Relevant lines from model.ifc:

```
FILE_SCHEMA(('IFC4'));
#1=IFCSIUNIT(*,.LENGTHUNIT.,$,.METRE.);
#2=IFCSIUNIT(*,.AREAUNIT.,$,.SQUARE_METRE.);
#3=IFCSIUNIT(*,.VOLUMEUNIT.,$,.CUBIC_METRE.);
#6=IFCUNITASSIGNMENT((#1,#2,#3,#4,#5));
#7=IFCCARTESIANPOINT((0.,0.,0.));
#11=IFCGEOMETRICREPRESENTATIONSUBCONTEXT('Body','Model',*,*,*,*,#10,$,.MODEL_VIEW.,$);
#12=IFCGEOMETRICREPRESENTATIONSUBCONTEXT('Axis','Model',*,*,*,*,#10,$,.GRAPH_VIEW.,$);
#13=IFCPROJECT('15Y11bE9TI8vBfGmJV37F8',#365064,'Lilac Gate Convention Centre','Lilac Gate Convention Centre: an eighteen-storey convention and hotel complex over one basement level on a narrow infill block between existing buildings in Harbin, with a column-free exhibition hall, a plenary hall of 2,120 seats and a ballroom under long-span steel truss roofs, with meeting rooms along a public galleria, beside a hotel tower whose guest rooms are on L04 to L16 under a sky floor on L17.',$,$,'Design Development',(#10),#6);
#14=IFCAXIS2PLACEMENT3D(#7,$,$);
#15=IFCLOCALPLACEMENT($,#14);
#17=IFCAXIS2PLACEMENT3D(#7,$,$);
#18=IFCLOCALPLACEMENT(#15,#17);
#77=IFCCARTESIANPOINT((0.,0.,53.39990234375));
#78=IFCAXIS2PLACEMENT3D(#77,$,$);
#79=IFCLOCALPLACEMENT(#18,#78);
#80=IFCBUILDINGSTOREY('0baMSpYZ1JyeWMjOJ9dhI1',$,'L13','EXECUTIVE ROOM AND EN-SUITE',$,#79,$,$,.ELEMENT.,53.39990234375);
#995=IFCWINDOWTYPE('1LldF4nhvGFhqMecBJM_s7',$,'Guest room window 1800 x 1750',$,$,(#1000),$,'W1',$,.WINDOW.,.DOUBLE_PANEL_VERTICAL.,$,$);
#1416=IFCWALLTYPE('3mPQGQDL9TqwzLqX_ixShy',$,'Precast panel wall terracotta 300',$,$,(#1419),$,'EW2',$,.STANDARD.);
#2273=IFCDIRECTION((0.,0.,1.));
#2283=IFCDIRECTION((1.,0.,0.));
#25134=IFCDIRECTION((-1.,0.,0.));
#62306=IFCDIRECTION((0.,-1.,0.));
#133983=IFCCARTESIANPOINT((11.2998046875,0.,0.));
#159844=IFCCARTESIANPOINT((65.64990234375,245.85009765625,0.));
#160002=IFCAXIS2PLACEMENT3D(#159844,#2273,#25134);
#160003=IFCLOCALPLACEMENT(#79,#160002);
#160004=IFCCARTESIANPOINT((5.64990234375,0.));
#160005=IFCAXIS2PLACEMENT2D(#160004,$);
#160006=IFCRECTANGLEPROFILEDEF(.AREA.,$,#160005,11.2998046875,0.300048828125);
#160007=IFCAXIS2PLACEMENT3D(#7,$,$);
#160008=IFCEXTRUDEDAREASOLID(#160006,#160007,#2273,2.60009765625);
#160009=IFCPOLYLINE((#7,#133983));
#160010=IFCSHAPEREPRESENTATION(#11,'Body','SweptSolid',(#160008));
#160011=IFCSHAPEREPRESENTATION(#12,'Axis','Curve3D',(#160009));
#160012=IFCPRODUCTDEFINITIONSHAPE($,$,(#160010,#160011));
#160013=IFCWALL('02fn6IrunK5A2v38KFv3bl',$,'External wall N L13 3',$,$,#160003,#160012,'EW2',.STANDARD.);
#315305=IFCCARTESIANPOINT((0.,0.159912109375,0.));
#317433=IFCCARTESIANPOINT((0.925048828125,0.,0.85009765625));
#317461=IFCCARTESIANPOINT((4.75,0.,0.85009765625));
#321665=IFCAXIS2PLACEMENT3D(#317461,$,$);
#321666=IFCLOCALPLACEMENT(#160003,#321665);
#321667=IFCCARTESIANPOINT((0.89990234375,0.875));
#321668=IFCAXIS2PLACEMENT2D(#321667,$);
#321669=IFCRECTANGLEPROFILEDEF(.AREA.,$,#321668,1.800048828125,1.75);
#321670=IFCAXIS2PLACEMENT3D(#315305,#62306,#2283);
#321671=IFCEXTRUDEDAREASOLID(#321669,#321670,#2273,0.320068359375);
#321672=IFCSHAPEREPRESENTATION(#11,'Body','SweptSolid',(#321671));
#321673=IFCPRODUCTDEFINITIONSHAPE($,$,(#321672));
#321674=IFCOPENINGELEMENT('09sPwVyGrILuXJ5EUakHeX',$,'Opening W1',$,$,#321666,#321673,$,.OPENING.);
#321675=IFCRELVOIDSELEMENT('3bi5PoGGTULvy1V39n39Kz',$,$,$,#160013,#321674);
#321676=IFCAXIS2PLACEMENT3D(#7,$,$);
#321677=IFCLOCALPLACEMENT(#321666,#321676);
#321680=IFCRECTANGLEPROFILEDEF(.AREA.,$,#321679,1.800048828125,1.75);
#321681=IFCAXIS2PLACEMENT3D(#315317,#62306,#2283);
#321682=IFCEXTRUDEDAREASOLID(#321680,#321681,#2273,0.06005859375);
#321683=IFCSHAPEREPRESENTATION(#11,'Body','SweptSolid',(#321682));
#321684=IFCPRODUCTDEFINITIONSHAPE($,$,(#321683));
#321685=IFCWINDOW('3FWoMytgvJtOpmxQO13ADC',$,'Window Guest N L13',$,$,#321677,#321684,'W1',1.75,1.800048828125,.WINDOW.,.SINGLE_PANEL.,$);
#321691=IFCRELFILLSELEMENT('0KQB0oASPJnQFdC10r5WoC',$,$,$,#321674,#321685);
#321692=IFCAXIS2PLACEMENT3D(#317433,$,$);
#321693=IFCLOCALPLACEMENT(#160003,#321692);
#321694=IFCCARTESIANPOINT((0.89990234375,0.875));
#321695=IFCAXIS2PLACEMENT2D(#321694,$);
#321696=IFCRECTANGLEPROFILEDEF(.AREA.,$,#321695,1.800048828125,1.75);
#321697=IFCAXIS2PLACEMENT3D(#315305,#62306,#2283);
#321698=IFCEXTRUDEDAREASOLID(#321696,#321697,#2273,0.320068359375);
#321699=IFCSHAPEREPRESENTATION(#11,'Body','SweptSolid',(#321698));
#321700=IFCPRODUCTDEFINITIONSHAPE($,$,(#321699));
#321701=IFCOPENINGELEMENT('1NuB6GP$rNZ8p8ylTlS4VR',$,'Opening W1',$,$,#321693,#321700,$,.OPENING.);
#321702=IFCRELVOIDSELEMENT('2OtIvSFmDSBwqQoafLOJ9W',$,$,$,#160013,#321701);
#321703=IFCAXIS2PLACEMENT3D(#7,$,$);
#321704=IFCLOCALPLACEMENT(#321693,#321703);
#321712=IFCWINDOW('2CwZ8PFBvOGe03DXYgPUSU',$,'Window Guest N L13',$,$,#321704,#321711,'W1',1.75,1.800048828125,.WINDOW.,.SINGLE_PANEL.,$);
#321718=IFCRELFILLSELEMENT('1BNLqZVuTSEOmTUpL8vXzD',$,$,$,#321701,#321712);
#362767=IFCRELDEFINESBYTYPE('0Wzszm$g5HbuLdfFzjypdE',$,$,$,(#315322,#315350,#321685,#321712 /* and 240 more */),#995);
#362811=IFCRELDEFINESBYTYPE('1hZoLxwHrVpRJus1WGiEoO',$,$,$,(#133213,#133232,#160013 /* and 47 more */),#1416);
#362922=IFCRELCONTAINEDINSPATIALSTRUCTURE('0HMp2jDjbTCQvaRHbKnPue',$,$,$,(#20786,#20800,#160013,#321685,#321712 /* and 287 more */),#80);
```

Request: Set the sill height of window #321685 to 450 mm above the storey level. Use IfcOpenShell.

```python
import numpy as np
import ifcopenshell
import ifcopenshell.api.geometry
import ifcopenshell.geom
import ifcopenshell.util.element
import ifcopenshell.util.placement
import ifcopenshell.util.shape
import ifcopenshell.util.unit

model = ifcopenshell.open("model.ifc")
unit_scale = ifcopenshell.util.unit.calculate_unit_scale(model)

window = model.by_id(321685)
opening = window.FillsVoids[0].RelatingOpeningElement
storey = ifcopenshell.util.element.get_container(window, ifc_class="IfcBuildingStorey")
level = ifcopenshell.util.placement.get_local_placement(storey.ObjectPlacement)[2, 3]

# The opening's origin need not be at the sill, so measure its lowest point.
shape = ifcopenshell.geom.create_shape(ifcopenshell.geom.settings(), opening)
bottom = ifcopenshell.util.shape.get_shape_bottom_elevation(shape, shape.geometry) / unit_scale
dz = level + 0.45 - bottom

shift = np.array([0.0, 0.0, dz])
# The window is placed relative to its opening, so it follows when the opening moves.
matrix = ifcopenshell.util.placement.get_local_placement(opening.ObjectPlacement)
matrix[:3, 3] += shift
ifcopenshell.api.geometry.edit_object_placement(
    model, product=opening, matrix=matrix, is_si=False, should_transform_children=True
)

print(f"moved by {dz * unit_scale:+.3f} m")

model.write("model_edited.ifc")
```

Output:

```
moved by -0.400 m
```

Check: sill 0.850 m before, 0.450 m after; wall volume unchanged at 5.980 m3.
